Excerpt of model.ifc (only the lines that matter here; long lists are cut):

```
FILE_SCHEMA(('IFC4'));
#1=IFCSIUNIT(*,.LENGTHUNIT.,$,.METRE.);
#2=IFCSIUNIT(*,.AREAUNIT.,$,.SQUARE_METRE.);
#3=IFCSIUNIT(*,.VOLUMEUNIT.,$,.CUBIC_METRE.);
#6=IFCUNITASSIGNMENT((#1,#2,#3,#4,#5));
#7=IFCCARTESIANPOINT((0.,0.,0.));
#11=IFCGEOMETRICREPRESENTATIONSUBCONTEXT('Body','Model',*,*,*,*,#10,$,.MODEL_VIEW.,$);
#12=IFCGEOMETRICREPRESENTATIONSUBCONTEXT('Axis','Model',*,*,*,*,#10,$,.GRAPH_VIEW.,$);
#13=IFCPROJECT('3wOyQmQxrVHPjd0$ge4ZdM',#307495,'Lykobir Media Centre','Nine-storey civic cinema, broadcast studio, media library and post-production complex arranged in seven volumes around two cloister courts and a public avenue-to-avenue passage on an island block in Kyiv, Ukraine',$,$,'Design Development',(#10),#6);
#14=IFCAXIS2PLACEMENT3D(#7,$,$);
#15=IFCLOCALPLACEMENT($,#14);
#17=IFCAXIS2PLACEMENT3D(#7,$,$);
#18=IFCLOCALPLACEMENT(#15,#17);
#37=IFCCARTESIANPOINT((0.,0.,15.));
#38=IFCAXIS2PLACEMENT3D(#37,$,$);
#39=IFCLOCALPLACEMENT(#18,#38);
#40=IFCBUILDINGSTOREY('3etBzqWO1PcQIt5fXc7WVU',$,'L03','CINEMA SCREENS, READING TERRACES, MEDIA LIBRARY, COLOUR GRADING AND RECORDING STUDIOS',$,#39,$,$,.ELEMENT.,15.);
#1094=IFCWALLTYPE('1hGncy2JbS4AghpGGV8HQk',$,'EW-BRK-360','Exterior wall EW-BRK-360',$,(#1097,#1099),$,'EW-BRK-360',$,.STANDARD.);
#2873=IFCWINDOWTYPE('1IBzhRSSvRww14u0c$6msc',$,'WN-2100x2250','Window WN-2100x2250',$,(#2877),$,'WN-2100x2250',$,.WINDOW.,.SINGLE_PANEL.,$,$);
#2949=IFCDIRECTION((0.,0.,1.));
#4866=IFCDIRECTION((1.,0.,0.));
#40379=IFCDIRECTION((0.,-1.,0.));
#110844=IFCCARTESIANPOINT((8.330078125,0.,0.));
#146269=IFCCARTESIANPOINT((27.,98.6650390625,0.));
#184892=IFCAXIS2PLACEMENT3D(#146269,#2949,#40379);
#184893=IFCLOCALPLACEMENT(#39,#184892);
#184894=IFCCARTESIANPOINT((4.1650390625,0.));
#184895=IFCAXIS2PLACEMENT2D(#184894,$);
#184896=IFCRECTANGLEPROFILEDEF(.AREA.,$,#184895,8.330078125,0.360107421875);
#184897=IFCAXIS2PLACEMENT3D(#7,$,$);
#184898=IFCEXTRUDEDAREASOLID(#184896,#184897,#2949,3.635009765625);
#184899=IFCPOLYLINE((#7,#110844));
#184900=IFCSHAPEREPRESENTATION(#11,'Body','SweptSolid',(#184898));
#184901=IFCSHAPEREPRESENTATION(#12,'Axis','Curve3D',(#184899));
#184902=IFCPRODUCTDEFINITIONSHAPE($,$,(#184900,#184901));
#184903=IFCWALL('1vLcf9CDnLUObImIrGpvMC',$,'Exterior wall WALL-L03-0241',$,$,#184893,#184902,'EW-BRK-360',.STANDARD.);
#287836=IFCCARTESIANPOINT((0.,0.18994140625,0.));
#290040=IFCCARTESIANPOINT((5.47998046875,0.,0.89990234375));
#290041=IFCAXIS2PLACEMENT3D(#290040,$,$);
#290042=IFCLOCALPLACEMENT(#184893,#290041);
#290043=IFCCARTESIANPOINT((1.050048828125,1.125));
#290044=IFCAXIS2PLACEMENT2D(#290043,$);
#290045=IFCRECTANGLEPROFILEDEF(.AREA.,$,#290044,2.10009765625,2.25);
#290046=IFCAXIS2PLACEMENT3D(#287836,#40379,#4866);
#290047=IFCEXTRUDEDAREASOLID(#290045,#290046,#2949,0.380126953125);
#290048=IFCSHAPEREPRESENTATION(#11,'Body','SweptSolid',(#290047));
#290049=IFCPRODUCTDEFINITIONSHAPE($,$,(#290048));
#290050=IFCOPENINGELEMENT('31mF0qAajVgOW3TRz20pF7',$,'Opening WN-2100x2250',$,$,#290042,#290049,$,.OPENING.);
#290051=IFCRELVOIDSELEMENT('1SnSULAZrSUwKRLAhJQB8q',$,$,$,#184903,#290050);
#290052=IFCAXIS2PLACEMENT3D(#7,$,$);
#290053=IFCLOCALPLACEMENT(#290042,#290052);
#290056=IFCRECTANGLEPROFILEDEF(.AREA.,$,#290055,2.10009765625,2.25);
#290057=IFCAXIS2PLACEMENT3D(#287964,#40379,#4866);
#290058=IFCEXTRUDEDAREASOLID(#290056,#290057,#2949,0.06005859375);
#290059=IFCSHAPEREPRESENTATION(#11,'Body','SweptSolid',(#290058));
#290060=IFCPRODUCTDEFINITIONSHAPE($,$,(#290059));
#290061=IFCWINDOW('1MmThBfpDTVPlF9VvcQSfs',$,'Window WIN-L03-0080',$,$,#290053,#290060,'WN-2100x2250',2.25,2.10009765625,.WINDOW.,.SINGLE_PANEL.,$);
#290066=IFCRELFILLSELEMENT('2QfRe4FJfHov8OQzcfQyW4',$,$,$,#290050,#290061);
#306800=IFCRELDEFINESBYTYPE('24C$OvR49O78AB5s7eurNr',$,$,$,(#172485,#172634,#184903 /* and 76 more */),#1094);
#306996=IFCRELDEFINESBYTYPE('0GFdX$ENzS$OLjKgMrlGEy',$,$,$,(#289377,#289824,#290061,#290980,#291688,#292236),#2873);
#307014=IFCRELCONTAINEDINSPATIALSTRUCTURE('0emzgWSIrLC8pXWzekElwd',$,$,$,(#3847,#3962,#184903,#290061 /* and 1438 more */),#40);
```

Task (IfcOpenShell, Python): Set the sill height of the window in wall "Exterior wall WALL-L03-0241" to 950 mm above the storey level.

```python
import numpy as np
import ifcopenshell
import ifcopenshell.api.geometry
import ifcopenshell.geom
import ifcopenshell.util.element
import ifcopenshell.util.placement
import ifcopenshell.util.shape
import ifcopenshell.util.unit

model = ifcopenshell.open("model.ifc")
unit_scale = ifcopenshell.util.unit.calculate_unit_scale(model)

window = model.by_guid("1MmThBfpDTVPlF9VvcQSfs")
opening = window.FillsVoids[0].RelatingOpeningElement
storey = ifcopenshell.util.element.get_container(window, ifc_class="IfcBuildingStorey")
level = ifcopenshell.util.placement.get_local_placement(storey.ObjectPlacement)[2, 3]

# The opening's origin need not be at the sill, so measure its lowest point.
shape = ifcopenshell.geom.create_shape(ifcopenshell.geom.settings(), opening)
bottom = ifcopenshell.util.shape.get_shape_bottom_elevation(shape, shape.geometry) / unit_scale
dz = level + 0.95 / unit_scale - bottom

shift = np.array([0.0, 0.0, dz])
# The window is placed relative to its opening, so it follows when the opening moves.
matrix = ifcopenshell.util.placement.get_local_placement(opening.ObjectPlacement)
matrix[:3, 3] += shift
ifcopenshell.api.geometry.edit_object_placement(
    model, product=opening, matrix=matrix, is_si=False, should_transform_children=True
)

print(f"moved by {dz * unit_scale:+.3f} m")

model.write("model_updated.ifc")
```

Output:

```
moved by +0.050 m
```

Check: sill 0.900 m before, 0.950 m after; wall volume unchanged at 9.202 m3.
